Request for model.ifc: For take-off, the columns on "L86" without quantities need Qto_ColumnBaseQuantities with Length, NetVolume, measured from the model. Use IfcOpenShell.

First a look at what the model holds.

```python
import ifcopenshell
import ifcopenshell.util.element
import ifcopenshell.util.unit

model = ifcopenshell.open("model.ifc")
print(model.schema)
for unit_type in ("LENGTHUNIT", "AREAUNIT", "VOLUMEUNIT"):
    print(unit_type, ifcopenshell.util.unit.calculate_unit_scale(model, unit_type))
storey = next(s for s in model.by_type("IfcBuildingStorey") if s.Name == "L86")
columns = [e for e in ifcopenshell.util.element.get_decomposition(storey) if e.is_a("IfcColumn")]
for e in sorted(columns, key=lambda e: e.id()):
    print(e.id(), e.is_a(), e.Name, list(ifcopenshell.util.element.get_psets(e, qtos_only=True)), sep=" | ")
```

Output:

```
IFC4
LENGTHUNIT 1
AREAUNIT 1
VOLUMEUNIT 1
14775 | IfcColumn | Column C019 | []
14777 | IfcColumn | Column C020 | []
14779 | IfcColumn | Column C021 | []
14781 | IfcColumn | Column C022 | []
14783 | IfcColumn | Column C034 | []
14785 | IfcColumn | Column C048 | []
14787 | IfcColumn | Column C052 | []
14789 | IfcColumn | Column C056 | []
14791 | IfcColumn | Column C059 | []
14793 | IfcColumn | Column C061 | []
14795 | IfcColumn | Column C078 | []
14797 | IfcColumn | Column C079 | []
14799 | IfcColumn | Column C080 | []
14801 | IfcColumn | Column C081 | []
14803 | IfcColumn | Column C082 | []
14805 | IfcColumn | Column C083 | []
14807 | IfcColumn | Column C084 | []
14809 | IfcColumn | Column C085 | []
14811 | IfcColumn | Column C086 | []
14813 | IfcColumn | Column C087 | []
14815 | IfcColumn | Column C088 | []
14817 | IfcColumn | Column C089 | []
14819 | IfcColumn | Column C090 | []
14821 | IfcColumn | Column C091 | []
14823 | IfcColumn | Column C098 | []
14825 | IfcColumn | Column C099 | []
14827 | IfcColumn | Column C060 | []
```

```python
import ifcopenshell
import ifcopenshell.api.pset
import ifcopenshell.geom
import ifcopenshell.util.element
import ifcopenshell.util.shape
import ifcopenshell.util.unit

model = ifcopenshell.open("model.ifc")
unit_scale = ifcopenshell.util.unit.calculate_unit_scale(model)
volume_scale = ifcopenshell.util.unit.calculate_unit_scale(model, "VOLUMEUNIT")
settings = ifcopenshell.geom.settings()

storey = next(s for s in model.by_type("IfcBuildingStorey") if s.Name == "L86")
columns = [e for e in ifcopenshell.util.element.get_decomposition(storey) if e.is_a("IfcColumn")]

for e in sorted(columns, key=lambda e: e.id()):
    if ifcopenshell.util.element.get_psets(e, qtos_only=True, should_inherit=False):
        continue
    # Geometry comes back in metres, in the element's own axes.
    shape = ifcopenshell.geom.create_shape(settings, e)
    values = {
        "Length": ifcopenshell.util.shape.get_z(shape.geometry) / unit_scale,
        "NetVolume": ifcopenshell.util.shape.get_volume(shape.geometry) / volume_scale,
    }
    qto = ifcopenshell.api.pset.add_qto(model, product=e, name="Qto_ColumnBaseQuantities")
    ifcopenshell.api.pset.edit_qto(model, qto=qto, properties=values)
    print(e.id(), {k: round(v, 3) for k, v in values.items()})

model.write("model_updated.ifc")
```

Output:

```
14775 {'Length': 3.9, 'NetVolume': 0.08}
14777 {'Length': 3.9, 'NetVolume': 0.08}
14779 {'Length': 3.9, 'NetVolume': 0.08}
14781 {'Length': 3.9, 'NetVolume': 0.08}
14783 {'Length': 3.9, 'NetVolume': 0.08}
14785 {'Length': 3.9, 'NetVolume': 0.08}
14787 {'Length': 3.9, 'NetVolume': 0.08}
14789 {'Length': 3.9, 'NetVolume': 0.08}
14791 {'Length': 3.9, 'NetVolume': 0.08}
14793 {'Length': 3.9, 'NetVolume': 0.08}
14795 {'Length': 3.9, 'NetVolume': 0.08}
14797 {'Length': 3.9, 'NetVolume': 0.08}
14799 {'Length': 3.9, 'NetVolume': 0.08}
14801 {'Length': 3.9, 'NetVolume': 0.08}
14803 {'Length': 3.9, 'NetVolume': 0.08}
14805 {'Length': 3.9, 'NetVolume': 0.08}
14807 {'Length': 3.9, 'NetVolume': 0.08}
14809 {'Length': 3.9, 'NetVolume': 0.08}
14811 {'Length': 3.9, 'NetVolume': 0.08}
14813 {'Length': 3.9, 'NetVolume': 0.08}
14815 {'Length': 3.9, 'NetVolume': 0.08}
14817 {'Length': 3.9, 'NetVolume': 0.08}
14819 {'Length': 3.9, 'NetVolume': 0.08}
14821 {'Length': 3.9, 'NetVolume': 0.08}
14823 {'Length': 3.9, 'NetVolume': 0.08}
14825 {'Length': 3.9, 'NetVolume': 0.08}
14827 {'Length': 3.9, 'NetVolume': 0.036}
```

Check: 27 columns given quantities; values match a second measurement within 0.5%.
